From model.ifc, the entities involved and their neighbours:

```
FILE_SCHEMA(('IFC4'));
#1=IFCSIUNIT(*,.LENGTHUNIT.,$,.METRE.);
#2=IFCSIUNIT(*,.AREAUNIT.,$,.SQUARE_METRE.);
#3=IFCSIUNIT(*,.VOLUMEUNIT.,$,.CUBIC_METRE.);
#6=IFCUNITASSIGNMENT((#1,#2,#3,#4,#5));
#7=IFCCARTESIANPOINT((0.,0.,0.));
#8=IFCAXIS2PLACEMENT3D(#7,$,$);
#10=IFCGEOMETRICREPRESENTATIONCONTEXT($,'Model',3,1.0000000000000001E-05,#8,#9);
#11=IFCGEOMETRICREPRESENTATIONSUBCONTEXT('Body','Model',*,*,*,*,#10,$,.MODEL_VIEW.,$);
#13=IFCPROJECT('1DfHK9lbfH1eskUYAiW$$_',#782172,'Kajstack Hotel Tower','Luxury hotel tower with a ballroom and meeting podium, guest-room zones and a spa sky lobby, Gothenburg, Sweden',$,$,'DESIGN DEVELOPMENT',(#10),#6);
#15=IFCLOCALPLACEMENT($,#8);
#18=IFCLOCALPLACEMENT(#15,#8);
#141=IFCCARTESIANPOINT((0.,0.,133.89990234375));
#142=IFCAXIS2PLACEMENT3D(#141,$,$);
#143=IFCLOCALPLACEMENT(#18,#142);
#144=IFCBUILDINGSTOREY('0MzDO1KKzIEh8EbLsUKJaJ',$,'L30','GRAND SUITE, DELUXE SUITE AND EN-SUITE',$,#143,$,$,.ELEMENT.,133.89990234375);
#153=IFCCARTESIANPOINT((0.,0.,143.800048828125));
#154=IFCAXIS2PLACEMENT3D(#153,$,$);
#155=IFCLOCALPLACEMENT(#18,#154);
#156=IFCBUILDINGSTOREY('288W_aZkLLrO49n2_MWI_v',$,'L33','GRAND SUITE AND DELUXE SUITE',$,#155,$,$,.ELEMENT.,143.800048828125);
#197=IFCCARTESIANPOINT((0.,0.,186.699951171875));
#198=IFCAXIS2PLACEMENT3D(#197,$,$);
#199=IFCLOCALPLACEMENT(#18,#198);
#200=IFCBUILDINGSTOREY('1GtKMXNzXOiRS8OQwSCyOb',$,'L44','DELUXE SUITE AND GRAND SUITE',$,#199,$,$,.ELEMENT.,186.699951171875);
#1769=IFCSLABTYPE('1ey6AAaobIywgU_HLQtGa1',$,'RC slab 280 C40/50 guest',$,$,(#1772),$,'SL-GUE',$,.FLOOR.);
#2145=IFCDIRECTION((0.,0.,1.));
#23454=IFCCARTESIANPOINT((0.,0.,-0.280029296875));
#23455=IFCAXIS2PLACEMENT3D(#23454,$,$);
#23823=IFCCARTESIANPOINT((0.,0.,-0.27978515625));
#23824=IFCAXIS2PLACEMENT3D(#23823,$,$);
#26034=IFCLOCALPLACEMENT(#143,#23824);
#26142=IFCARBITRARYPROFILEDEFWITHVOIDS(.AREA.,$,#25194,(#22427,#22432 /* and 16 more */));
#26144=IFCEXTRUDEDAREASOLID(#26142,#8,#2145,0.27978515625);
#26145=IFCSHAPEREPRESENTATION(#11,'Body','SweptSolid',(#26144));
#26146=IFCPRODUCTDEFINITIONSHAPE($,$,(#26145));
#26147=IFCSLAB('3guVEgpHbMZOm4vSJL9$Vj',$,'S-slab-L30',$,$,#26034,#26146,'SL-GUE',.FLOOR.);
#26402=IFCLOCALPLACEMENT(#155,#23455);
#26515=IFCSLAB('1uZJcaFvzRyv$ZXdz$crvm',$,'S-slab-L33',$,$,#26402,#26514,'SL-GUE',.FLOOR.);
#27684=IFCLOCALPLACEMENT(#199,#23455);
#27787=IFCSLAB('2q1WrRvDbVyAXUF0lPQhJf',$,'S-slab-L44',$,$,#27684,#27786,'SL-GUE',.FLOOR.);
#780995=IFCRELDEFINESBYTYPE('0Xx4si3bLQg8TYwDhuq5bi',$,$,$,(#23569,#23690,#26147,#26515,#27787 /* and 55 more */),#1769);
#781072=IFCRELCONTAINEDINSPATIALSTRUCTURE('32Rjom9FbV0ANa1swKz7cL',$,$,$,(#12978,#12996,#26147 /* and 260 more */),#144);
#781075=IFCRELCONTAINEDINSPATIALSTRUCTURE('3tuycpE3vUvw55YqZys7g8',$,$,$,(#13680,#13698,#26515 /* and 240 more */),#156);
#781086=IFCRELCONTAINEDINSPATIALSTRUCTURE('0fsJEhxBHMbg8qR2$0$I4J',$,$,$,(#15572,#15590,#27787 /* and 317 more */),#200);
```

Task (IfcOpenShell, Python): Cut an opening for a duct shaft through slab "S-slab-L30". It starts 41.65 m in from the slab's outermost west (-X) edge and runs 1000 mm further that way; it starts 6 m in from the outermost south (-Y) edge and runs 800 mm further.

```python
import numpy as np
import ifcopenshell
import ifcopenshell.api.feature
import ifcopenshell.api.geometry
import ifcopenshell.api.root
import ifcopenshell.geom
import ifcopenshell.util.placement
import ifcopenshell.util.representation
import ifcopenshell.util.shape
import ifcopenshell.util.unit

model = ifcopenshell.open("model.ifc")
unit_scale = ifcopenshell.util.unit.calculate_unit_scale(model)
settings = ifcopenshell.geom.settings()


def volume(element):
    """Net volume in cubic metres, openings subtracted."""
    shape = ifcopenshell.geom.create_shape(settings, element)
    return ifcopenshell.util.shape.get_volume(shape.geometry)


slab = model.by_guid("3guVEgpHbMZOm4vSJL9$Vj")
before = volume(slab)

# Extent in the slab's own axes, in metres. The edges named are its -X and -Y sides.
slab_shape = ifcopenshell.geom.create_shape(settings, slab)
vertices = ifcopenshell.util.shape.get_vertices(slab_shape.geometry)
x_min, y_min, bottom = vertices.min(axis=0)
top = vertices[:, 2].max()

opening = ifcopenshell.api.root.create_entity(model, ifc_class="IfcOpeningElement", name="Duct shaft opening", predefined_type="OPENING")
context = ifcopenshell.util.representation.get_context(model, "Model", "Body", "MODEL_VIEW")
width, depth = 1, 0.8
outline = [(0.0, 0.0), (width, 0.0), (width, depth), (0.0, depth), (0.0, 0.0)]
# Overshoot both faces by 50 mm so the cut is clean.
shape = ifcopenshell.api.geometry.add_slab_representation(
    model, context=context, depth=top - bottom + 0.1, polyline=outline
)
ifcopenshell.api.geometry.assign_representation(model, product=opening, representation=shape)

matrix = ifcopenshell.util.placement.get_local_placement(slab.ObjectPlacement)
matrix[:, 3] = matrix @ np.append(np.array([x_min + 41.65, y_min + 6, bottom - 0.05]) / unit_scale, 1.0)
ifcopenshell.api.geometry.edit_object_placement(model, product=opening, matrix=matrix, is_si=False)
ifcopenshell.api.feature.add_feature(model, feature=opening, element=slab)

after = volume(slab)

print(f"slab volume {before:.3f} -> {after:.3f} m3")

model.write("model_updated.ifc")
```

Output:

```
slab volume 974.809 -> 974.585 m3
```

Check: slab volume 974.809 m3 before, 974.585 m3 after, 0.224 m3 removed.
